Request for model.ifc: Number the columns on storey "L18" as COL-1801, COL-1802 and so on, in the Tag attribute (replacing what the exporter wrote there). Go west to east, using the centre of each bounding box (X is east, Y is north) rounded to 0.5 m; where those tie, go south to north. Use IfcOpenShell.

First a look at what the model holds.

```python
import ifcopenshell
import ifcopenshell.util.element
import ifcopenshell.util.placement

model = ifcopenshell.open("model.ifc")
print(model.schema)
storey = next(s for s in model.by_type("IfcBuildingStorey") if s.Name == "L18")
columns = [e for e in ifcopenshell.util.element.get_decomposition(storey) if e.is_a("IfcColumn")]
for e in sorted(columns, key=lambda e: e.id()):
    origin = ifcopenshell.util.placement.get_local_placement(e.ObjectPlacement)[:3, 3]
    print(e.id(), e.Tag, e.Name, origin.round(2) + 0.0, sep=" | ")
```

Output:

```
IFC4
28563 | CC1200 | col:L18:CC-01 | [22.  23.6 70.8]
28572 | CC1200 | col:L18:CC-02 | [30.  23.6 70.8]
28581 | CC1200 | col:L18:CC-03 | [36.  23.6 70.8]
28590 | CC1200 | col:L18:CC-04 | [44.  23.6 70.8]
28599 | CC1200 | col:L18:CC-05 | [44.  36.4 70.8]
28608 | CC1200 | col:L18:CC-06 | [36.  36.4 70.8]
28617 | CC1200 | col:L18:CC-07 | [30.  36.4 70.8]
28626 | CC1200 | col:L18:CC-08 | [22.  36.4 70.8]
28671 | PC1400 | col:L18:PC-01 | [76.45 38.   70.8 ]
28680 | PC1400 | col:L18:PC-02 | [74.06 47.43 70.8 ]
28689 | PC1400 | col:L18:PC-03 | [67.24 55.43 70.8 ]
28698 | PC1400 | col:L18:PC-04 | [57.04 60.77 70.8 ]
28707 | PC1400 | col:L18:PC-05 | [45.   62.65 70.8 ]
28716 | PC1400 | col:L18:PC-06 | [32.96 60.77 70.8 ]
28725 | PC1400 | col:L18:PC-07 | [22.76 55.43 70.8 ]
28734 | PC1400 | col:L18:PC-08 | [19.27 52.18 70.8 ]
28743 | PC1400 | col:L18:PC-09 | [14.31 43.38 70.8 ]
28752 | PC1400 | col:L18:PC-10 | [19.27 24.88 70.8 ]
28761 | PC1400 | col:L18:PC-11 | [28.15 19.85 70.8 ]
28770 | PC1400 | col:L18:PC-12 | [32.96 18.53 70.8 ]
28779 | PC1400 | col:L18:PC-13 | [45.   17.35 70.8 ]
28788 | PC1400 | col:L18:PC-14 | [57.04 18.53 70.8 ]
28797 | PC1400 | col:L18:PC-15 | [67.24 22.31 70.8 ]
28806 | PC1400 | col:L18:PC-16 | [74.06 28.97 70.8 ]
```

```python
import ifcopenshell
import ifcopenshell.geom
import ifcopenshell.util.element
import ifcopenshell.util.shape

model = ifcopenshell.open("model.ifc")
settings = ifcopenshell.geom.settings()
settings.set("use-world-coords", True)


def centre(element):
    shape = ifcopenshell.geom.create_shape(settings, element)
    return ifcopenshell.util.shape.get_bbox_centroid(shape.geometry)


storey = next(s for s in model.by_type("IfcBuildingStorey") if s.Name == "L18")
columns = [e for e in ifcopenshell.util.element.get_decomposition(storey) if e.is_a("IfcColumn")]

# Insertion points can sit at a corner or the storey origin, so sort by the geometry (in metres).
centres = {e: centre(e) for e in columns}
columns.sort(key=lambda e: (round(centres[e][0] / 0.5), centres[e][1]))

for i, e in enumerate(columns, start=1):
    number = f"COL-18{i:02d}"
    e.Tag = number
    print(e.id(), number)

model.write("model_updated.ifc")
```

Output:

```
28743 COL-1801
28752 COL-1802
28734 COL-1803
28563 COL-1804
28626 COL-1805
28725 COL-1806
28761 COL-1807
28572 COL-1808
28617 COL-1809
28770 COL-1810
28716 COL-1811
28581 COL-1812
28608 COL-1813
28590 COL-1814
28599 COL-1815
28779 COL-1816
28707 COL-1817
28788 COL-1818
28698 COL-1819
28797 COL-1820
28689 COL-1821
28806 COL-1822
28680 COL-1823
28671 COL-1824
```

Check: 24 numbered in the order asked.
